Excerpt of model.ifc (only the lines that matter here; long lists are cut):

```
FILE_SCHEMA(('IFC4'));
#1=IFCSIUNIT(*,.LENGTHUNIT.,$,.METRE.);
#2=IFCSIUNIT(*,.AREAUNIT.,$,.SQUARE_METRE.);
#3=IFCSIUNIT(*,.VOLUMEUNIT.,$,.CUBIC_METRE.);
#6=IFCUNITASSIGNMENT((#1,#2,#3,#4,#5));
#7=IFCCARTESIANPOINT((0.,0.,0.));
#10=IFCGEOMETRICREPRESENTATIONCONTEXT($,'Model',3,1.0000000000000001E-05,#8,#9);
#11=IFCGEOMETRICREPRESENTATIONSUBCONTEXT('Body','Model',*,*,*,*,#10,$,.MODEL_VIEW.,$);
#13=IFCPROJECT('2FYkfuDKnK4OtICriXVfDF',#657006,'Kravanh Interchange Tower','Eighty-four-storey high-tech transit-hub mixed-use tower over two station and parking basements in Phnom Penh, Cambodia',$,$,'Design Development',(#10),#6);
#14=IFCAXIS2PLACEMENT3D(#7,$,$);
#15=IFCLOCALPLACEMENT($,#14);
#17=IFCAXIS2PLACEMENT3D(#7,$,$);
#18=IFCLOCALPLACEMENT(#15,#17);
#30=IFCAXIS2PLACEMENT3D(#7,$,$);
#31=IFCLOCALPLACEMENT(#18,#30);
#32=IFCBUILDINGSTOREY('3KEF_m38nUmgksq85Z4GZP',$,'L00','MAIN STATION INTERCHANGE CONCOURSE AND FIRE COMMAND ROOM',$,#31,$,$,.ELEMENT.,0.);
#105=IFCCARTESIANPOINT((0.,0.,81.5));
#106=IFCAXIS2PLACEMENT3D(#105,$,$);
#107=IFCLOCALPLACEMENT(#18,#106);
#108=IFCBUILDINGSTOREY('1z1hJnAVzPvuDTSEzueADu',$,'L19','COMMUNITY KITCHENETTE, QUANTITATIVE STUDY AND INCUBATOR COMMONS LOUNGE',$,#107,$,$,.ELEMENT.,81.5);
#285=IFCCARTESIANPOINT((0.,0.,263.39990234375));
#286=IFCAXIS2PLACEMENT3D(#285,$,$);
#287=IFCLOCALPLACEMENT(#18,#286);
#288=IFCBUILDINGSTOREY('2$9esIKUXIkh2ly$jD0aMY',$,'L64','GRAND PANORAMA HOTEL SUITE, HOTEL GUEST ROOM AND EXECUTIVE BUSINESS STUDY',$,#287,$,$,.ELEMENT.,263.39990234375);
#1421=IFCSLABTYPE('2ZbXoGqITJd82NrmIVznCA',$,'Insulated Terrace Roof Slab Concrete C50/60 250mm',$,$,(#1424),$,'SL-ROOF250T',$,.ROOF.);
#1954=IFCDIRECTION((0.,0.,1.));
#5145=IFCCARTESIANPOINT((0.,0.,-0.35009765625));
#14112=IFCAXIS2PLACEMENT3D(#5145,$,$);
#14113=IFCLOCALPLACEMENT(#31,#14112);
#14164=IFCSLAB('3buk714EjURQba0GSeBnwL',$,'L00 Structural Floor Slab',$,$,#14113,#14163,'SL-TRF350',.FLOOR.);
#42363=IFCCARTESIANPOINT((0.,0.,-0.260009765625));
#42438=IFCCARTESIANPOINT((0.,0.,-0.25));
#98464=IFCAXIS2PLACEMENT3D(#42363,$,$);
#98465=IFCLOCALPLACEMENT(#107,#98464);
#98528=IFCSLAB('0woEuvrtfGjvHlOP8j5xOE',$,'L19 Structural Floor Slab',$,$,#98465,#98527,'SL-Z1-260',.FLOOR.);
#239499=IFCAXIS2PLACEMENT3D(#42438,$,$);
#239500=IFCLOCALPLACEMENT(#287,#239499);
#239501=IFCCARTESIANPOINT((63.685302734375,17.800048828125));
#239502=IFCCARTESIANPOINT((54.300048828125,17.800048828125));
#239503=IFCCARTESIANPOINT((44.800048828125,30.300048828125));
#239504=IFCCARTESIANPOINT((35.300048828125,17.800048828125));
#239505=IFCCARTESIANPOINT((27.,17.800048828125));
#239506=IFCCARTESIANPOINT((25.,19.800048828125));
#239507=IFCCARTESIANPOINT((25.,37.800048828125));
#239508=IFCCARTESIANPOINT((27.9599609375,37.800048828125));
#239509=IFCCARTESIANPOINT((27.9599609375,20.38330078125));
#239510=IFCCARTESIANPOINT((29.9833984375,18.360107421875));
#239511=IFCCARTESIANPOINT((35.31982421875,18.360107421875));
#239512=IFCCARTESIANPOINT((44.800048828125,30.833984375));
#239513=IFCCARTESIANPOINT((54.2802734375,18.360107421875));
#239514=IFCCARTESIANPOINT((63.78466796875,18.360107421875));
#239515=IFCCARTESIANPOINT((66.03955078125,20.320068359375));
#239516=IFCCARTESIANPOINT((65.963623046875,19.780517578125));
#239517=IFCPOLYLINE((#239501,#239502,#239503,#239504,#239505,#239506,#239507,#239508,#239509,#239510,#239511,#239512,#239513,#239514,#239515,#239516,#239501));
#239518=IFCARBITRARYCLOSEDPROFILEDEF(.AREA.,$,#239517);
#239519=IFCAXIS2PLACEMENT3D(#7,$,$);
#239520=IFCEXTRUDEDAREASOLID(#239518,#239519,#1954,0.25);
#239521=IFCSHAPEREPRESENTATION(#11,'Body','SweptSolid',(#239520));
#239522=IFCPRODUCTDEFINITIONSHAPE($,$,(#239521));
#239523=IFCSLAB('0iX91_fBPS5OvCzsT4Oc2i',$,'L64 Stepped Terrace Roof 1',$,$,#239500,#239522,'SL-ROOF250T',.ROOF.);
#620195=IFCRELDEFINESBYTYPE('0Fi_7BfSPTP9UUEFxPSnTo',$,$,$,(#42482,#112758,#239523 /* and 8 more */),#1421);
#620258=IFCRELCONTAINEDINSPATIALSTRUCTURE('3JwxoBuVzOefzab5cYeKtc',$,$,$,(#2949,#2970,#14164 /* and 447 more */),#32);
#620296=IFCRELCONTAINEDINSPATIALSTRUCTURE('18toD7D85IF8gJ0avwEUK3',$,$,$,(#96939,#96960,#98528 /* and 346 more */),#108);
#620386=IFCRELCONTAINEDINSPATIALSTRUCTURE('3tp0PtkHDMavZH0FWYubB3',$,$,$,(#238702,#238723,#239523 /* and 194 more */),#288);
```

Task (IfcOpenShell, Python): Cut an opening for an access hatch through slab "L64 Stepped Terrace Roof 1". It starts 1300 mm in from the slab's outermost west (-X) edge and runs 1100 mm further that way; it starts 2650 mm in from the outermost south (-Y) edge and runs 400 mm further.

```python
import numpy as np
import ifcopenshell
import ifcopenshell.api.feature
import ifcopenshell.api.geometry
import ifcopenshell.api.root
import ifcopenshell.geom
import ifcopenshell.util.placement
import ifcopenshell.util.representation
import ifcopenshell.util.shape
import ifcopenshell.util.unit

model = ifcopenshell.open("model.ifc")
unit_scale = ifcopenshell.util.unit.calculate_unit_scale(model)
settings = ifcopenshell.geom.settings()


def volume(element):
    """Net volume in cubic metres, openings subtracted."""
    shape = ifcopenshell.geom.create_shape(settings, element)
    return ifcopenshell.util.shape.get_volume(shape.geometry)


slab = model.by_guid("0iX91_fBPS5OvCzsT4Oc2i")
before = volume(slab)

# Extent in the slab's own axes, in metres. The edges named are its -X and -Y sides.
slab_shape = ifcopenshell.geom.create_shape(settings, slab)
vertices = ifcopenshell.util.shape.get_vertices(slab_shape.geometry)
x_min, y_min, bottom = vertices.min(axis=0)
top = vertices[:, 2].max()

opening = ifcopenshell.api.root.create_entity(model, ifc_class="IfcOpeningElement", name="Access hatch opening", predefined_type="OPENING")
context = ifcopenshell.util.representation.get_context(model, "Model", "Body", "MODEL_VIEW")
width, depth = 1.1, 0.4
outline = [(0.0, 0.0), (width, 0.0), (width, depth), (0.0, depth), (0.0, 0.0)]
# Overshoot both faces by 50 mm so the cut is clean.
shape = ifcopenshell.api.geometry.add_slab_representation(
    model, context=context, depth=top - bottom + 0.1, polyline=outline
)
ifcopenshell.api.geometry.assign_representation(model, product=opening, representation=shape)

matrix = ifcopenshell.util.placement.get_local_placement(slab.ObjectPlacement)
matrix[:, 3] = matrix @ np.append(np.array([x_min + 1.3, y_min + 2.65, bottom - 0.05]) / unit_scale, 1.0)
ifcopenshell.api.geometry.edit_object_placement(model, product=opening, matrix=matrix, is_si=False)
ifcopenshell.api.feature.add_feature(model, feature=opening, element=slab)

after = volume(slab)

print(f"slab volume {before:.3f} -> {after:.3f} m3")

model.write("model_updated.ifc")
```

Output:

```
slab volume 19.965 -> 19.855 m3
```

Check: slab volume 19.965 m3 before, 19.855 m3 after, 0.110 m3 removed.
